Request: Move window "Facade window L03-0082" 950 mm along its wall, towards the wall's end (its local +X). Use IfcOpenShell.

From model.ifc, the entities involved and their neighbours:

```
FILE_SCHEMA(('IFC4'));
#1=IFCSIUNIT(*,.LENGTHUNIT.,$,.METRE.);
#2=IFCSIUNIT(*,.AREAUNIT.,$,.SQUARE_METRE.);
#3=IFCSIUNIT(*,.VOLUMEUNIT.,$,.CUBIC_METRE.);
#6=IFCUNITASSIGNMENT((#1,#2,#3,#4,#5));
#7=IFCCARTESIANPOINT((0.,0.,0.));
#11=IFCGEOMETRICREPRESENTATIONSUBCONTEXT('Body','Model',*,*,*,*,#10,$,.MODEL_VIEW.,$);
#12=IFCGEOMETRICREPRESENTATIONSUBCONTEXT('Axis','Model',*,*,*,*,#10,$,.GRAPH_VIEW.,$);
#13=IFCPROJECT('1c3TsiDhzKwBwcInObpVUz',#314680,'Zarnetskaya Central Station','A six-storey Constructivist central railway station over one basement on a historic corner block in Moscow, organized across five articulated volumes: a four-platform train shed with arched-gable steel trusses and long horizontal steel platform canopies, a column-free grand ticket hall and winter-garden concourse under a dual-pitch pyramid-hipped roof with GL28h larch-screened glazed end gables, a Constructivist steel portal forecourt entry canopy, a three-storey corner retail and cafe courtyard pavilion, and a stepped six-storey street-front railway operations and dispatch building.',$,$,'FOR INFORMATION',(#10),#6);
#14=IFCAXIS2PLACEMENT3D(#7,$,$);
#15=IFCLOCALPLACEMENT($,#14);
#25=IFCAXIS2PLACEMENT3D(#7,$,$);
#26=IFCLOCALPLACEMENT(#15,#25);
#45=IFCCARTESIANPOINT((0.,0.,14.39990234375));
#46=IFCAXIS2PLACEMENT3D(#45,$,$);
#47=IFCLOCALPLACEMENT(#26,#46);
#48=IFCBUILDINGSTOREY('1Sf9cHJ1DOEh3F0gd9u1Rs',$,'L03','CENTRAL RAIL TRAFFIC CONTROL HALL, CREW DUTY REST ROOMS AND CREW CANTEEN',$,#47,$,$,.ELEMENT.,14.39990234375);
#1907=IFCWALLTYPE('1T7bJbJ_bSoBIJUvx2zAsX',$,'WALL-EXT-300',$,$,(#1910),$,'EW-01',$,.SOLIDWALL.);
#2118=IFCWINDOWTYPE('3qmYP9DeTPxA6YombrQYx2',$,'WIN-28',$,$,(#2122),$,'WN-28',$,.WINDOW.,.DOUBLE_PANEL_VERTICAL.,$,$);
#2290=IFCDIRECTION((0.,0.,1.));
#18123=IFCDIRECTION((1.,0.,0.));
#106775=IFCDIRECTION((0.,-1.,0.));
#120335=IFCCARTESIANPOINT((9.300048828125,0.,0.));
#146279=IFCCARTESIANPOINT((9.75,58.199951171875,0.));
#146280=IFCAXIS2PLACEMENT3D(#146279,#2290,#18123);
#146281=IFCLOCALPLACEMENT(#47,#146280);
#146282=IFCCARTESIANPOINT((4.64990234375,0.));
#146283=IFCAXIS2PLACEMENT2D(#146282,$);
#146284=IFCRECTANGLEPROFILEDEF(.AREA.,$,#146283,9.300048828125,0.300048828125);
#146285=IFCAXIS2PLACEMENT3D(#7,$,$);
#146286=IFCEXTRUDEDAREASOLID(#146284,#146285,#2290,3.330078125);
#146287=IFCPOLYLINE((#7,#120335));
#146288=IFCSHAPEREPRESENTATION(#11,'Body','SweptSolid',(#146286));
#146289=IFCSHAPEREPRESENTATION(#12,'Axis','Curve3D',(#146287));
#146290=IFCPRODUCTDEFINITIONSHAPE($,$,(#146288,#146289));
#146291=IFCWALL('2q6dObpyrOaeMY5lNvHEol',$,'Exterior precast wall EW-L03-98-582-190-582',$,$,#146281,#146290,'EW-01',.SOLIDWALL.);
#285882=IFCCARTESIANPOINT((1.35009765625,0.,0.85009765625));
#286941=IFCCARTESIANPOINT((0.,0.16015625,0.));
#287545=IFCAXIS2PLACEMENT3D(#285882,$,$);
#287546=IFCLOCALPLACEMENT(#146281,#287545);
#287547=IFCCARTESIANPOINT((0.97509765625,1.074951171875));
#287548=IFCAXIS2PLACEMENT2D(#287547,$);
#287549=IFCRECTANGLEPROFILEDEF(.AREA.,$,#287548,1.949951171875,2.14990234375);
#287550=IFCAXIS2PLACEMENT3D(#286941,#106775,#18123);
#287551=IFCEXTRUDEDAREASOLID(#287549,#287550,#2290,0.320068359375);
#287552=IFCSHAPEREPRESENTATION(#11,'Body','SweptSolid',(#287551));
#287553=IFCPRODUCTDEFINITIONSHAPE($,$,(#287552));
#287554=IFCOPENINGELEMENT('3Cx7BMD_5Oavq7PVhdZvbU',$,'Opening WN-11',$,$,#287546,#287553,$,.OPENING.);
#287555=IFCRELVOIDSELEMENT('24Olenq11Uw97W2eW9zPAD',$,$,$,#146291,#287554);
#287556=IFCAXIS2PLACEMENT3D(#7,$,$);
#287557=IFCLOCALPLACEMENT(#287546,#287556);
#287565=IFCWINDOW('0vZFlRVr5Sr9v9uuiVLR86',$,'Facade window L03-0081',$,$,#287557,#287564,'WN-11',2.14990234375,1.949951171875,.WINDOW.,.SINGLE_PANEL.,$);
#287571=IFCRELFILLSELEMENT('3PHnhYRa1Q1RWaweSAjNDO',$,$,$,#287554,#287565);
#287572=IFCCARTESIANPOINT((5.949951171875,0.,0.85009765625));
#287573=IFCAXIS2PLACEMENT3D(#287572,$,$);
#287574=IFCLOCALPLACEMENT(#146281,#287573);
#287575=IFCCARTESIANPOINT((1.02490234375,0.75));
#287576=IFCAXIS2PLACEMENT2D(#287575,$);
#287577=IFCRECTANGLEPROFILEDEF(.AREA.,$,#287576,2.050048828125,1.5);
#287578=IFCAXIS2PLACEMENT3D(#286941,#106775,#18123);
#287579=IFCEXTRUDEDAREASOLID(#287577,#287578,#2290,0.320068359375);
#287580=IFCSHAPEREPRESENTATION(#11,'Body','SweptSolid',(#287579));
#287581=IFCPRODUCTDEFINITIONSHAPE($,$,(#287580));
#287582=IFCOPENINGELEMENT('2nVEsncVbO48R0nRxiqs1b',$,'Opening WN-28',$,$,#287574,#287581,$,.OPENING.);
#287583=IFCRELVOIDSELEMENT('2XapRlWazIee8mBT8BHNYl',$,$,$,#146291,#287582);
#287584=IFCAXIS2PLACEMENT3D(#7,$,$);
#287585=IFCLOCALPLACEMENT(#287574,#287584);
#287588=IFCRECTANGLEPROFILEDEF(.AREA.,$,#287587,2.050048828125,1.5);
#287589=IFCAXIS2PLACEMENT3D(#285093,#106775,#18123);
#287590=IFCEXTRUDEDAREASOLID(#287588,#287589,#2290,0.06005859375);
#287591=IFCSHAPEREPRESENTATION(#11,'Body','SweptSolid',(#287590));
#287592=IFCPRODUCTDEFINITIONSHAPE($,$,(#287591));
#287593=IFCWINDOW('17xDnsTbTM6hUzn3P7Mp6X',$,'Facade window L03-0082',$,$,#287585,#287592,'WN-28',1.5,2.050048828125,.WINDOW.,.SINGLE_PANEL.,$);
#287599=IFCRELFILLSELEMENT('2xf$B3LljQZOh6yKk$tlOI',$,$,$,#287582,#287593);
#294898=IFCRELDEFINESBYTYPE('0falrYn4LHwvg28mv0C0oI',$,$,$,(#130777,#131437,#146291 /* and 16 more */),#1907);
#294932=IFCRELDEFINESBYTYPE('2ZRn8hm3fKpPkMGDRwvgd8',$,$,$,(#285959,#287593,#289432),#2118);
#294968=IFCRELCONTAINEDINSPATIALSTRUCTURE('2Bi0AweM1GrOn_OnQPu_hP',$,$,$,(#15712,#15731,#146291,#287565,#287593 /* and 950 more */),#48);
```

```python
import ifcopenshell
import ifcopenshell.api.geometry
import ifcopenshell.util.placement
import ifcopenshell.util.unit

model = ifcopenshell.open("model.ifc")
unit_scale = ifcopenshell.util.unit.calculate_unit_scale(model)

window = model.by_id(287593)
opening = window.FillsVoids[0].RelatingOpeningElement
wall = opening.VoidsElements[0].RelatingBuildingElement

wall_matrix = ifcopenshell.util.placement.get_local_placement(wall.ObjectPlacement)
shift = wall_matrix[:3, 0] * 0.95 / unit_scale
before = ifcopenshell.util.placement.get_local_placement(window.ObjectPlacement)[:3, 3].copy()

# The window is placed relative to its opening, so it follows when the opening moves.
matrix = ifcopenshell.util.placement.get_local_placement(opening.ObjectPlacement)
matrix[:3, 3] += shift
ifcopenshell.api.geometry.edit_object_placement(
    model, product=opening, matrix=matrix, is_si=False, should_transform_children=True
)

after = ifcopenshell.util.placement.get_local_placement(window.ObjectPlacement)[:3, 3]
print("window moved by", (after - before).round(3) + 0.0)

model.write("model_updated.ifc")
```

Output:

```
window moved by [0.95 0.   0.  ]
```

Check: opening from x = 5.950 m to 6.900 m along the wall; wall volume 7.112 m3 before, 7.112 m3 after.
